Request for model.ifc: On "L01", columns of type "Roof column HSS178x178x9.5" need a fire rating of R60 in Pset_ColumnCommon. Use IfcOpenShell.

First a look at what the model holds.

```python
import ifcopenshell
import ifcopenshell.util.element

model = ifcopenshell.open("model.ifc")
print(model.schema)
storey = next(s for s in model.by_type("IfcBuildingStorey") if s.Name == "L01")
columns = [e for e in ifcopenshell.util.element.get_decomposition(storey) if e.is_a("IfcColumn")]
seen = {}
for e in columns:
    element_type = ifcopenshell.util.element.get_type(e)
    key = (element_type.Name if element_type != e and element_type else None, ifcopenshell.util.element.get_pset(e, "Pset_ColumnCommon", "FireRating"))
    seen[key] = seen.get(key, 0) + 1
for (name, value), count in sorted(seen.items(), key=str):
    print(count, "x", name, "|", value)
```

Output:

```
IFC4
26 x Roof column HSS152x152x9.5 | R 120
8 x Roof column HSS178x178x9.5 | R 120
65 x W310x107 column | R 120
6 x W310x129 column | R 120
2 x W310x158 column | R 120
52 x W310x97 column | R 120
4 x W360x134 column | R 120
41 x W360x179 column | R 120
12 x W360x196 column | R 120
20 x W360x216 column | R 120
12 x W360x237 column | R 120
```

```python
import ifcopenshell
import ifcopenshell.api.pset
import ifcopenshell.util.element

model = ifcopenshell.open("model.ifc")

storey = next(s for s in model.by_type("IfcBuildingStorey") if s.Name == "L01")
columns = [e for e in ifcopenshell.util.element.get_decomposition(storey) if e.is_a("IfcColumn")]

count = 0
for e in columns:
    element_type = ifcopenshell.util.element.get_type(e)
    if element_type in (None, e) or element_type.Name != "Roof column HSS178x178x9.5":
        continue
    # add_pset returns the element's existing set when there is one.
    pset = ifcopenshell.api.pset.add_pset(model, product=e, name="Pset_ColumnCommon")
    ifcopenshell.api.pset.edit_pset(model, pset=pset, properties={"FireRating": "R60"})
    count += 1

print(count, "columns updated")

model.write("model_edited.ifc")
```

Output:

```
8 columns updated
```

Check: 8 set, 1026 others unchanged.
